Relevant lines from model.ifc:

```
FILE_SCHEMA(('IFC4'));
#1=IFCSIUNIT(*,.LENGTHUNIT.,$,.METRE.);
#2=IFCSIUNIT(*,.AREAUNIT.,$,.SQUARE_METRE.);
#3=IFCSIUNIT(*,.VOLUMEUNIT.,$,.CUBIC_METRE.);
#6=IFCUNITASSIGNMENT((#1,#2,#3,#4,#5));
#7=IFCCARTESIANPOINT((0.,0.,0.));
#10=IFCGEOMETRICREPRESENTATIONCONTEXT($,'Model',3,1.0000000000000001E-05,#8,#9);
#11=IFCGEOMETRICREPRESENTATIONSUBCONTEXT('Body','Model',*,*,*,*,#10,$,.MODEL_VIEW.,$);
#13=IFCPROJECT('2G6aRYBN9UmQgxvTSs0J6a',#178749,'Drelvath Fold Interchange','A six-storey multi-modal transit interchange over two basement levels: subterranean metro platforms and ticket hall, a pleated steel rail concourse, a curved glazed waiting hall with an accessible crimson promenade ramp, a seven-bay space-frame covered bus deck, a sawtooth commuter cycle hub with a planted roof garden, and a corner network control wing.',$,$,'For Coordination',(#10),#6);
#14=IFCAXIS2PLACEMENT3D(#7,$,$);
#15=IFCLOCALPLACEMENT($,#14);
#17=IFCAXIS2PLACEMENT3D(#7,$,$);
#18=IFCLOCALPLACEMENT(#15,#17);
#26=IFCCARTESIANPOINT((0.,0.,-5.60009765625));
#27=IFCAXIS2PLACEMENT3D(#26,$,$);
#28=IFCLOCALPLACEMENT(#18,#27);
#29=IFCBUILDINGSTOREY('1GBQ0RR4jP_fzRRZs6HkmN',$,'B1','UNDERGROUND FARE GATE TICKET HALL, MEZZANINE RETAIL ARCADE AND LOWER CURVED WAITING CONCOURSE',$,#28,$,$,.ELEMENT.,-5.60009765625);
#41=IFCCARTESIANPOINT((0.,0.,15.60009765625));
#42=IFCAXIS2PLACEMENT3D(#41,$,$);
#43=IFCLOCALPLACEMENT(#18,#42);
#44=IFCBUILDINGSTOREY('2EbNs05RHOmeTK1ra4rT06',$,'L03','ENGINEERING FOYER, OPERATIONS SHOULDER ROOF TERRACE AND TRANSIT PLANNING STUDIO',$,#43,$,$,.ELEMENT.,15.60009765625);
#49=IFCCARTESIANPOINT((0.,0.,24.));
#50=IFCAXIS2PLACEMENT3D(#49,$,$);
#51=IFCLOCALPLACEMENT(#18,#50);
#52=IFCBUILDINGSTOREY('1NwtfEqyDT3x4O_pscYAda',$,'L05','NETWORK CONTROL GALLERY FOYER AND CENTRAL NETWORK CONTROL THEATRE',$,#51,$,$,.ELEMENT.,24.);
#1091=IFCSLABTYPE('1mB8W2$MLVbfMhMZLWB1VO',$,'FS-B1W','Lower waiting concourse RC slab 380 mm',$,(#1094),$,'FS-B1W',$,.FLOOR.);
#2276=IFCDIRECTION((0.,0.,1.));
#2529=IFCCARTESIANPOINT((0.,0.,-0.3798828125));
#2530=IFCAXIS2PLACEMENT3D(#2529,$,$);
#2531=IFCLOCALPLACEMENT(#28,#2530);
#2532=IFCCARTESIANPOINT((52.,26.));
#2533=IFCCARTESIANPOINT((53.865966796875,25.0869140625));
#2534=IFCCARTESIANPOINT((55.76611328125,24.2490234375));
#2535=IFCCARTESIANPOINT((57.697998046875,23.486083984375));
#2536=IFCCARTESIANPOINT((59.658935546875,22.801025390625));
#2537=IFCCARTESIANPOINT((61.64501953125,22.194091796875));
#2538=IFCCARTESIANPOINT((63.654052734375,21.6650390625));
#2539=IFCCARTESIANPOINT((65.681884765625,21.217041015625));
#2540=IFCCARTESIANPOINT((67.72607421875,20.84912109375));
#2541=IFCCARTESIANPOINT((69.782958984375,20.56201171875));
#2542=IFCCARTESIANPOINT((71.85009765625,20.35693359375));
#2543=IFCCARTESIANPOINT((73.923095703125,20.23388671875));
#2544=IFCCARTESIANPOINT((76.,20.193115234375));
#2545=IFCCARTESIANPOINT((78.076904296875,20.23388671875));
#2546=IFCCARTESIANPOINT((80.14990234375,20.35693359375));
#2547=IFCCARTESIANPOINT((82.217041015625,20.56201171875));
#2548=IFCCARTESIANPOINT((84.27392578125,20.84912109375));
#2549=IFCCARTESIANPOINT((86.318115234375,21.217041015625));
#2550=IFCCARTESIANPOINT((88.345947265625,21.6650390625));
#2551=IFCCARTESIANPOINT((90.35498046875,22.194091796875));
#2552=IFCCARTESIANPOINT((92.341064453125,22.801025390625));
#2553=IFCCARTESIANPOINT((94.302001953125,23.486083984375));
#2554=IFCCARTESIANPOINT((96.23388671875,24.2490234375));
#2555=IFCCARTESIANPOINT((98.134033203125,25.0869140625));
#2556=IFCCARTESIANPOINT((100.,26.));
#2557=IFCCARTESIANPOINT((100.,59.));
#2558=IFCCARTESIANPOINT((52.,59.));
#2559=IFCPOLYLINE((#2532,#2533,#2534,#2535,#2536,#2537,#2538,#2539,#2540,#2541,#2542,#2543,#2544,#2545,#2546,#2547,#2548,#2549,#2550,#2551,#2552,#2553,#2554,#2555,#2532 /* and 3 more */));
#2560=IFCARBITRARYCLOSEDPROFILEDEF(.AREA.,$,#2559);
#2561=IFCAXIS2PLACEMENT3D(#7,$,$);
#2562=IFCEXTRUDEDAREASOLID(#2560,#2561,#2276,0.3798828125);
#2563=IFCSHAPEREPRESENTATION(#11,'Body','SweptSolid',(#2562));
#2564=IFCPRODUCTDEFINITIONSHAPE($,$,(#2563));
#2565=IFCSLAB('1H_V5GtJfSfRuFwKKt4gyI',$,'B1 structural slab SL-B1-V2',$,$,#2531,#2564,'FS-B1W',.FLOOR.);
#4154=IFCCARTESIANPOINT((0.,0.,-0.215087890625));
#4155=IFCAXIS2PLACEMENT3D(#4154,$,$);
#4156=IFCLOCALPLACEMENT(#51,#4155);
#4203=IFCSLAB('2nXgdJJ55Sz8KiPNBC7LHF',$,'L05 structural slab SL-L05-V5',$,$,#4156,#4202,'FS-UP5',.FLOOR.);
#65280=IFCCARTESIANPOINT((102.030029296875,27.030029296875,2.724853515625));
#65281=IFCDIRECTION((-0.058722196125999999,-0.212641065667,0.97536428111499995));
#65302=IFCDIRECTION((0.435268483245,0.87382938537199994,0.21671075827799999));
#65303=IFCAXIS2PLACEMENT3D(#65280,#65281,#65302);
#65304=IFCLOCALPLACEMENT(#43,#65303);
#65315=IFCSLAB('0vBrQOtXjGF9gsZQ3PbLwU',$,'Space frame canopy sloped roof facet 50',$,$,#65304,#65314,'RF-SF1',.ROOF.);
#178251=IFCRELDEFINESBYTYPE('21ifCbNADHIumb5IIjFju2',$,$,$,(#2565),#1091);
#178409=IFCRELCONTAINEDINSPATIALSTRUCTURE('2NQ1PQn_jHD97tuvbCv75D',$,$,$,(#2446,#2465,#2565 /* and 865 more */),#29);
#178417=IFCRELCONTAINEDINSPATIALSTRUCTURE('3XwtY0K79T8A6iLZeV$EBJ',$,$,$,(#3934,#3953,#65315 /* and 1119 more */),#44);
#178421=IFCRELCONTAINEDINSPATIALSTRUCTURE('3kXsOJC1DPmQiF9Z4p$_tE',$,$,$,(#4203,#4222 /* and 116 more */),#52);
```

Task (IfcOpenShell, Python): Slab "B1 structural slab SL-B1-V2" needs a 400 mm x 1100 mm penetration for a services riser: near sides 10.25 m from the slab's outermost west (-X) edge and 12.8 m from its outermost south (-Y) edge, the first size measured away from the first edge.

```python
import numpy as np
import ifcopenshell
import ifcopenshell.api.feature
import ifcopenshell.api.geometry
import ifcopenshell.api.root
import ifcopenshell.geom
import ifcopenshell.util.placement
import ifcopenshell.util.representation
import ifcopenshell.util.shape
import ifcopenshell.util.unit

model = ifcopenshell.open("model.ifc")
unit_scale = ifcopenshell.util.unit.calculate_unit_scale(model)
settings = ifcopenshell.geom.settings()


def volume(element):
    """Net volume in cubic metres, openings subtracted."""
    shape = ifcopenshell.geom.create_shape(settings, element)
    return ifcopenshell.util.shape.get_volume(shape.geometry)


slab = model.by_guid("1H_V5GtJfSfRuFwKKt4gyI")
before = volume(slab)

# Extent in the slab's own axes, in metres. The edges named are its -X and -Y sides.
slab_shape = ifcopenshell.geom.create_shape(settings, slab)
vertices = ifcopenshell.util.shape.get_vertices(slab_shape.geometry)
x_min, y_min, bottom = vertices.min(axis=0)
top = vertices[:, 2].max()

opening = ifcopenshell.api.root.create_entity(model, ifc_class="IfcOpeningElement", name="Services riser opening", predefined_type="OPENING")
context = ifcopenshell.util.representation.get_context(model, "Model", "Body", "MODEL_VIEW")
width, depth = 0.4, 1.1
outline = [(0.0, 0.0), (width, 0.0), (width, depth), (0.0, depth), (0.0, 0.0)]
# Overshoot both faces by 50 mm so the cut is clean.
shape = ifcopenshell.api.geometry.add_slab_representation(
    model, context=context, depth=top - bottom + 0.1, polyline=outline
)
ifcopenshell.api.geometry.assign_representation(model, product=opening, representation=shape)

matrix = ifcopenshell.util.placement.get_local_placement(slab.ObjectPlacement)
matrix[:, 3] = matrix @ np.append(np.array([x_min + 10.25, y_min + 12.8, bottom - 0.05]) / unit_scale, 1.0)
ifcopenshell.api.geometry.edit_object_placement(model, product=opening, matrix=matrix, is_si=False)
ifcopenshell.api.feature.add_feature(model, feature=opening, element=slab)

after = volume(slab)

print(f"slab volume {before:.3f} -> {after:.3f} m3")

model.write("model_rev.ifc")
```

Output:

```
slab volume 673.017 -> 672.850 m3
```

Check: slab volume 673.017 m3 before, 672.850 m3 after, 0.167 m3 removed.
